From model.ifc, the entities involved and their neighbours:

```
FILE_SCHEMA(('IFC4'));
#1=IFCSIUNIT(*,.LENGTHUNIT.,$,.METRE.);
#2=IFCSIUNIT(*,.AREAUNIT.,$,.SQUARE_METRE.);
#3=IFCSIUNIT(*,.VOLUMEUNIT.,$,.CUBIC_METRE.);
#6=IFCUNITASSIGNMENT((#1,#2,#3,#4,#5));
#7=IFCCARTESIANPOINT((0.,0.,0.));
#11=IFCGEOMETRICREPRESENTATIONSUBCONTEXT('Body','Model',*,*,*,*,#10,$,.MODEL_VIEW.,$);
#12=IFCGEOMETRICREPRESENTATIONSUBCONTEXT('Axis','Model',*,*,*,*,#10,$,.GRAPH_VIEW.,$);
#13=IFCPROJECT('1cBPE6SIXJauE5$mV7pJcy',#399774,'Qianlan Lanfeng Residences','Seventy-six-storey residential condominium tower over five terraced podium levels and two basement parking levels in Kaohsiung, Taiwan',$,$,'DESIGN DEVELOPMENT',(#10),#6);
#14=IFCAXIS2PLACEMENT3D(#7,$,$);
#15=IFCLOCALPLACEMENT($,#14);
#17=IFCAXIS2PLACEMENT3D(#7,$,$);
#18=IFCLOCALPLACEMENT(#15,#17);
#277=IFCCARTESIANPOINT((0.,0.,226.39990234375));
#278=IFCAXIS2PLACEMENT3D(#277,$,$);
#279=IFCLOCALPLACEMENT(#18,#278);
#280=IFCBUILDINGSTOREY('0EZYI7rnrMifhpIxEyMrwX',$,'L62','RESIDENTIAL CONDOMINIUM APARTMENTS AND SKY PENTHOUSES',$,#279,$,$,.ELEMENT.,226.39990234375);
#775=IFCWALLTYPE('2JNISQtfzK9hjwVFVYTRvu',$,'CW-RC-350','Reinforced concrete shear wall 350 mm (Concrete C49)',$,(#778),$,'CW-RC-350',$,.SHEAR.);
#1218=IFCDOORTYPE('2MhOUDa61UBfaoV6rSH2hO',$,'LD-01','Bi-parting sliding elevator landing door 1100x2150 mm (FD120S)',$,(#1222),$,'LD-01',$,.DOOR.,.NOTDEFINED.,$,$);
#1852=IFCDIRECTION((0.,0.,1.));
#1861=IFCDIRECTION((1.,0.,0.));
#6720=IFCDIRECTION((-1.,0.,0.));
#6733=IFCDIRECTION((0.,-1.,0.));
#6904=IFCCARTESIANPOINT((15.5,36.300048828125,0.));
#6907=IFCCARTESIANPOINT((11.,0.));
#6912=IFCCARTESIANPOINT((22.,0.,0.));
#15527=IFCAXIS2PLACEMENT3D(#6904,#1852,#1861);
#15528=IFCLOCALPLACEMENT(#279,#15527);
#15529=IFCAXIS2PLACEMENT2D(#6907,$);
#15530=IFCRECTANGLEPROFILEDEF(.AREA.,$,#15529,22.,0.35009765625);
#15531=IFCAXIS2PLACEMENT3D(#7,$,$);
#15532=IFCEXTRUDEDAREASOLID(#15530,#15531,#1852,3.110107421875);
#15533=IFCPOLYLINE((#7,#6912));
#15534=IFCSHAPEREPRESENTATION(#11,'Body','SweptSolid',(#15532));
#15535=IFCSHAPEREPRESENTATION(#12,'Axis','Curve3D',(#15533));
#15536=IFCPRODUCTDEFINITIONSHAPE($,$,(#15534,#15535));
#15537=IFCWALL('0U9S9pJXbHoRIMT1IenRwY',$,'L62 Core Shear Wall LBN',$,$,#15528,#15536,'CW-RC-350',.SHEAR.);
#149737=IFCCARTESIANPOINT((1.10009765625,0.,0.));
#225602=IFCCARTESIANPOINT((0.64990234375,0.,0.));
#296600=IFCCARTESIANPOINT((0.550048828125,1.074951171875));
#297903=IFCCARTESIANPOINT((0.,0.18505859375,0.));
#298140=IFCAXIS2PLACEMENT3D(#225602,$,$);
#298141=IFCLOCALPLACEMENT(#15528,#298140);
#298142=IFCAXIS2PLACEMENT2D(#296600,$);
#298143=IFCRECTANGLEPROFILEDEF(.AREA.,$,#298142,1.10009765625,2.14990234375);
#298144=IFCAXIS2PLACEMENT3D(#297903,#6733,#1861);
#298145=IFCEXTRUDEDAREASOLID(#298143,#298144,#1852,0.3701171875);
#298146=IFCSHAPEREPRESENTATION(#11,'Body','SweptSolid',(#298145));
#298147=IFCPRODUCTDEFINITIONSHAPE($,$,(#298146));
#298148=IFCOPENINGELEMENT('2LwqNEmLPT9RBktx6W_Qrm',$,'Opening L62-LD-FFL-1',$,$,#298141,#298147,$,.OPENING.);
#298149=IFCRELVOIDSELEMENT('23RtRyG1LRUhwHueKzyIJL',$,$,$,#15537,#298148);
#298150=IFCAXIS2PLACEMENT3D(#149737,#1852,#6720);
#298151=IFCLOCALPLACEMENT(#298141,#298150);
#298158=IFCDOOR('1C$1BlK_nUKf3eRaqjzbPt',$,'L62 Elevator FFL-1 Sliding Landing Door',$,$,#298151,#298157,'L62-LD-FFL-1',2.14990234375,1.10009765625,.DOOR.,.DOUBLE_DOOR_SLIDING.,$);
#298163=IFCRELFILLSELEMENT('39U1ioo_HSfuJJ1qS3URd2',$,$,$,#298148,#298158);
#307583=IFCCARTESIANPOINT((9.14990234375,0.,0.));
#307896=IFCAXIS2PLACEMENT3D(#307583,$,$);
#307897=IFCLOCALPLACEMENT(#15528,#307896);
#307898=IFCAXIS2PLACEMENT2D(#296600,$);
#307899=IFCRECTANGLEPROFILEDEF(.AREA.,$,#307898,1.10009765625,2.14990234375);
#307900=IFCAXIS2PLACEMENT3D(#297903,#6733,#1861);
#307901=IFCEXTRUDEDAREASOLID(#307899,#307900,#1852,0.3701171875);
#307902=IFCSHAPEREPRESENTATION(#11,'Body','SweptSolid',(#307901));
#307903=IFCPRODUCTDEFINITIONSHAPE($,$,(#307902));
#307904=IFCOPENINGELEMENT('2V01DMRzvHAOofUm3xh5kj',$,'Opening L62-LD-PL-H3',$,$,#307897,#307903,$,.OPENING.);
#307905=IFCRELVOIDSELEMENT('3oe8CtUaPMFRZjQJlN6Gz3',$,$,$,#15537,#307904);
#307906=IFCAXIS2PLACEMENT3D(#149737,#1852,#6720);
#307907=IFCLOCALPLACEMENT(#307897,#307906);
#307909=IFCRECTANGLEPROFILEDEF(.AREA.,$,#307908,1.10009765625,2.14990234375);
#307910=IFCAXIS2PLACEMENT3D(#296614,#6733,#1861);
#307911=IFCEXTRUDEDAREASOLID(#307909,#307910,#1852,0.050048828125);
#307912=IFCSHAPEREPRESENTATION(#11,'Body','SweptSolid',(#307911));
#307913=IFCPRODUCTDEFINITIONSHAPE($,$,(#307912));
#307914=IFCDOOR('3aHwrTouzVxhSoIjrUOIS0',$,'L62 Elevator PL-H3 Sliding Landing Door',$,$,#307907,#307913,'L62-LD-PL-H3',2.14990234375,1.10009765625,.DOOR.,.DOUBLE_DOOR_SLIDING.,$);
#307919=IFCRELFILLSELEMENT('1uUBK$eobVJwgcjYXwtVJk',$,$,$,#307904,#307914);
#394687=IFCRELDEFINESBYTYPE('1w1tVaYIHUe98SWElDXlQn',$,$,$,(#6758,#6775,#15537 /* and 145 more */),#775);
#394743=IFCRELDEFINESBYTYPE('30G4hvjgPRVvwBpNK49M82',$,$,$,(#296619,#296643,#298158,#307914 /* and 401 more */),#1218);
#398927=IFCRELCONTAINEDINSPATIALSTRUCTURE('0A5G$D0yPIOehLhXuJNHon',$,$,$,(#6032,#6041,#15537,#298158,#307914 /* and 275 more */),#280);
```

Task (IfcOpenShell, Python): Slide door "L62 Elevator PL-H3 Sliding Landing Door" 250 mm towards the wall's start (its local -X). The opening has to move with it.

```python
import ifcopenshell
import ifcopenshell.api.geometry
import ifcopenshell.util.placement
import ifcopenshell.util.unit

model = ifcopenshell.open("model.ifc")
unit_scale = ifcopenshell.util.unit.calculate_unit_scale(model)

door = model.by_id(307914)
opening = door.FillsVoids[0].RelatingOpeningElement
wall = opening.VoidsElements[0].RelatingBuildingElement

wall_matrix = ifcopenshell.util.placement.get_local_placement(wall.ObjectPlacement)
shift = wall_matrix[:3, 0] * -0.25 / unit_scale
before = ifcopenshell.util.placement.get_local_placement(door.ObjectPlacement)[:3, 3].copy()

# The door is placed relative to its opening, so it follows when the opening moves.
matrix = ifcopenshell.util.placement.get_local_placement(opening.ObjectPlacement)
matrix[:3, 3] += shift
ifcopenshell.api.geometry.edit_object_placement(
    model, product=opening, matrix=matrix, is_si=False, should_transform_children=True
)

after = ifcopenshell.util.placement.get_local_placement(door.ObjectPlacement)[:3, 3]
print("door moved by", (after - before).round(3) + 0.0)

model.write("model_edited.ifc")
```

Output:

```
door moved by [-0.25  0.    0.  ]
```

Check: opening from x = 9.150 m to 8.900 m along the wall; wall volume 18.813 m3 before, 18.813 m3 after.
